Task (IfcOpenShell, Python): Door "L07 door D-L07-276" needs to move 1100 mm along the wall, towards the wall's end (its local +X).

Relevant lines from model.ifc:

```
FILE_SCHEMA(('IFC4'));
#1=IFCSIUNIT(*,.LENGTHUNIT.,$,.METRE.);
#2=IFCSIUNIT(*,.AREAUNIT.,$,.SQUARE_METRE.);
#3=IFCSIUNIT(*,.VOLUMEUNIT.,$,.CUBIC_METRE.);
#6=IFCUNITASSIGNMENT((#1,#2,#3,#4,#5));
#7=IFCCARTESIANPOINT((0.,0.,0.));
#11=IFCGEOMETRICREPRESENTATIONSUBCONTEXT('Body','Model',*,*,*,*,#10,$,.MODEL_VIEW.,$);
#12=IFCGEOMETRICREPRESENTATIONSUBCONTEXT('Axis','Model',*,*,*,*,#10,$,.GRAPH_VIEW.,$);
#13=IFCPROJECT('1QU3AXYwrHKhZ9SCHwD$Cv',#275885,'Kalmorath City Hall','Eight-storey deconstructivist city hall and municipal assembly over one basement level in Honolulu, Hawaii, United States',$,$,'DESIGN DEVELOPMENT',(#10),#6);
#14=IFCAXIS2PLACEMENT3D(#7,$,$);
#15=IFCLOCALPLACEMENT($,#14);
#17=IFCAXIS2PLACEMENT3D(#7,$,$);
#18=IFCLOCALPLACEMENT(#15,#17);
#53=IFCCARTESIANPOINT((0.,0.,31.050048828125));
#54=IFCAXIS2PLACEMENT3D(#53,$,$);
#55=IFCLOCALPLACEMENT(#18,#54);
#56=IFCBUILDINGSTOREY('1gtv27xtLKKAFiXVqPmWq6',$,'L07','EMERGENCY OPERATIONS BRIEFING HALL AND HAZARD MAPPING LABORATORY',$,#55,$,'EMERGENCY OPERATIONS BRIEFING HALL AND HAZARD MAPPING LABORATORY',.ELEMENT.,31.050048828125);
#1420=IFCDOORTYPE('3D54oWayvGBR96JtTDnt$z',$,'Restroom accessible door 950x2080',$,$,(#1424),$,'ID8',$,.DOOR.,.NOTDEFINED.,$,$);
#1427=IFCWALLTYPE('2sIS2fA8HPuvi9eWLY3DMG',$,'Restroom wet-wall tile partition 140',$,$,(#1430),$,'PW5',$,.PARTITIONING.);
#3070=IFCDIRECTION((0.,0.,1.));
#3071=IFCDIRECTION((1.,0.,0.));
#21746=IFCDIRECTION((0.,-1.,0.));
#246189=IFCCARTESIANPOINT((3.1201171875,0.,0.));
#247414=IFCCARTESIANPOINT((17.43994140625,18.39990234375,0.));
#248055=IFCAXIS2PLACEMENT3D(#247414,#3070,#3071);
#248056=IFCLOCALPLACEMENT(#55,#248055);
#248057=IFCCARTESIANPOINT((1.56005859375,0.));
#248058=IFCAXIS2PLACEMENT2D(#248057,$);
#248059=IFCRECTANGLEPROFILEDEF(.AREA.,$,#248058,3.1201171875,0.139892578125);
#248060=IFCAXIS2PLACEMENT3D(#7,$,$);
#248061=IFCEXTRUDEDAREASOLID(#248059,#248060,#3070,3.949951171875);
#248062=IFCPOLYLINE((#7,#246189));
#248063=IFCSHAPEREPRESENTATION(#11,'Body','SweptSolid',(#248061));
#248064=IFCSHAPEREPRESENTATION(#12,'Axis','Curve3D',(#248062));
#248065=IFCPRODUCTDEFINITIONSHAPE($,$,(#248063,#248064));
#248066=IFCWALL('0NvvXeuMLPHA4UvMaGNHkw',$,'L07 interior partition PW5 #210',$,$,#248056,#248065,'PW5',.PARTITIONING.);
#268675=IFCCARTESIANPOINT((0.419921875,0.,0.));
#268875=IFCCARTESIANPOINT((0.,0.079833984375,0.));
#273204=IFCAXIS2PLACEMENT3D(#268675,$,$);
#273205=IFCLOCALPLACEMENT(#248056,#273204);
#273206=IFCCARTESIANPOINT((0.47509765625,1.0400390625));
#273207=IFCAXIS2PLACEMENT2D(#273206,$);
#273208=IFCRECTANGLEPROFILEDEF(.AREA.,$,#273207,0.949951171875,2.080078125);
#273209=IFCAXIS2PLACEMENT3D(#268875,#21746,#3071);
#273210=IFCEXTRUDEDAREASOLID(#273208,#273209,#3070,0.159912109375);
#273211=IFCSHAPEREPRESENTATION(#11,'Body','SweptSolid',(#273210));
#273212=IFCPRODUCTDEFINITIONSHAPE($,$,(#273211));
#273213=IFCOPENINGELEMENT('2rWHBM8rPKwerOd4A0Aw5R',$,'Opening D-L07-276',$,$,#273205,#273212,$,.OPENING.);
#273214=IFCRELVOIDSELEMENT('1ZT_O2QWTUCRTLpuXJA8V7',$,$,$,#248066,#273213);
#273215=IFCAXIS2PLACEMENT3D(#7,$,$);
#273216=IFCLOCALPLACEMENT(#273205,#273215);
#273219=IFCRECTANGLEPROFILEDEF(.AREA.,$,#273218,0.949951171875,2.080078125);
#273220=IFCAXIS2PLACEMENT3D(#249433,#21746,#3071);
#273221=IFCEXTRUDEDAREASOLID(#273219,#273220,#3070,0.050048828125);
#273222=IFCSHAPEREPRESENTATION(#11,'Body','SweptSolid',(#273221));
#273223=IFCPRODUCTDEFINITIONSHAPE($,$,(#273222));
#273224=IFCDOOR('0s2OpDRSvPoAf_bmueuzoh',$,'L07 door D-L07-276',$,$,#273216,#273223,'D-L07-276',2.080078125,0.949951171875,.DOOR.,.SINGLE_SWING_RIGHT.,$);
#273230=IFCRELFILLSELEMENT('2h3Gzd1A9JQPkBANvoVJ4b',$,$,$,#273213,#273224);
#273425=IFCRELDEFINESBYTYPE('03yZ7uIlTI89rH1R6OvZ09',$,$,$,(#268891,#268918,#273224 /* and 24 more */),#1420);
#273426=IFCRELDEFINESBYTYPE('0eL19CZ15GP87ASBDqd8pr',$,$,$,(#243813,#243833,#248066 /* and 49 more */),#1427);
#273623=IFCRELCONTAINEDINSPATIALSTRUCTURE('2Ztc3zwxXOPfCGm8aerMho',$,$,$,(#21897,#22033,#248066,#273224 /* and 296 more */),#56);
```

```python
import ifcopenshell
import ifcopenshell.api.geometry
import ifcopenshell.util.placement

model = ifcopenshell.open("model.ifc")

door = model.by_guid("0s2OpDRSvPoAf_bmueuzoh")
opening = door.FillsVoids[0].RelatingOpeningElement
wall = opening.VoidsElements[0].RelatingBuildingElement

wall_matrix = ifcopenshell.util.placement.get_local_placement(wall.ObjectPlacement)
shift = wall_matrix[:3, 0] * 1.1
before = ifcopenshell.util.placement.get_local_placement(door.ObjectPlacement)[:3, 3].copy()

# The door is placed relative to its opening, so it follows when the opening moves.
matrix = ifcopenshell.util.placement.get_local_placement(opening.ObjectPlacement)
matrix[:3, 3] += shift
ifcopenshell.api.geometry.edit_object_placement(
    model, product=opening, matrix=matrix, is_si=False, should_transform_children=True
)

after = ifcopenshell.util.placement.get_local_placement(door.ObjectPlacement)[:3, 3]
print("door moved by", (after - before).round(3) + 0.0)

model.write("model-out.ifc")
```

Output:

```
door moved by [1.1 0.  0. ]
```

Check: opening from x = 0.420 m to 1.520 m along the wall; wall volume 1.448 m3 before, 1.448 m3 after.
